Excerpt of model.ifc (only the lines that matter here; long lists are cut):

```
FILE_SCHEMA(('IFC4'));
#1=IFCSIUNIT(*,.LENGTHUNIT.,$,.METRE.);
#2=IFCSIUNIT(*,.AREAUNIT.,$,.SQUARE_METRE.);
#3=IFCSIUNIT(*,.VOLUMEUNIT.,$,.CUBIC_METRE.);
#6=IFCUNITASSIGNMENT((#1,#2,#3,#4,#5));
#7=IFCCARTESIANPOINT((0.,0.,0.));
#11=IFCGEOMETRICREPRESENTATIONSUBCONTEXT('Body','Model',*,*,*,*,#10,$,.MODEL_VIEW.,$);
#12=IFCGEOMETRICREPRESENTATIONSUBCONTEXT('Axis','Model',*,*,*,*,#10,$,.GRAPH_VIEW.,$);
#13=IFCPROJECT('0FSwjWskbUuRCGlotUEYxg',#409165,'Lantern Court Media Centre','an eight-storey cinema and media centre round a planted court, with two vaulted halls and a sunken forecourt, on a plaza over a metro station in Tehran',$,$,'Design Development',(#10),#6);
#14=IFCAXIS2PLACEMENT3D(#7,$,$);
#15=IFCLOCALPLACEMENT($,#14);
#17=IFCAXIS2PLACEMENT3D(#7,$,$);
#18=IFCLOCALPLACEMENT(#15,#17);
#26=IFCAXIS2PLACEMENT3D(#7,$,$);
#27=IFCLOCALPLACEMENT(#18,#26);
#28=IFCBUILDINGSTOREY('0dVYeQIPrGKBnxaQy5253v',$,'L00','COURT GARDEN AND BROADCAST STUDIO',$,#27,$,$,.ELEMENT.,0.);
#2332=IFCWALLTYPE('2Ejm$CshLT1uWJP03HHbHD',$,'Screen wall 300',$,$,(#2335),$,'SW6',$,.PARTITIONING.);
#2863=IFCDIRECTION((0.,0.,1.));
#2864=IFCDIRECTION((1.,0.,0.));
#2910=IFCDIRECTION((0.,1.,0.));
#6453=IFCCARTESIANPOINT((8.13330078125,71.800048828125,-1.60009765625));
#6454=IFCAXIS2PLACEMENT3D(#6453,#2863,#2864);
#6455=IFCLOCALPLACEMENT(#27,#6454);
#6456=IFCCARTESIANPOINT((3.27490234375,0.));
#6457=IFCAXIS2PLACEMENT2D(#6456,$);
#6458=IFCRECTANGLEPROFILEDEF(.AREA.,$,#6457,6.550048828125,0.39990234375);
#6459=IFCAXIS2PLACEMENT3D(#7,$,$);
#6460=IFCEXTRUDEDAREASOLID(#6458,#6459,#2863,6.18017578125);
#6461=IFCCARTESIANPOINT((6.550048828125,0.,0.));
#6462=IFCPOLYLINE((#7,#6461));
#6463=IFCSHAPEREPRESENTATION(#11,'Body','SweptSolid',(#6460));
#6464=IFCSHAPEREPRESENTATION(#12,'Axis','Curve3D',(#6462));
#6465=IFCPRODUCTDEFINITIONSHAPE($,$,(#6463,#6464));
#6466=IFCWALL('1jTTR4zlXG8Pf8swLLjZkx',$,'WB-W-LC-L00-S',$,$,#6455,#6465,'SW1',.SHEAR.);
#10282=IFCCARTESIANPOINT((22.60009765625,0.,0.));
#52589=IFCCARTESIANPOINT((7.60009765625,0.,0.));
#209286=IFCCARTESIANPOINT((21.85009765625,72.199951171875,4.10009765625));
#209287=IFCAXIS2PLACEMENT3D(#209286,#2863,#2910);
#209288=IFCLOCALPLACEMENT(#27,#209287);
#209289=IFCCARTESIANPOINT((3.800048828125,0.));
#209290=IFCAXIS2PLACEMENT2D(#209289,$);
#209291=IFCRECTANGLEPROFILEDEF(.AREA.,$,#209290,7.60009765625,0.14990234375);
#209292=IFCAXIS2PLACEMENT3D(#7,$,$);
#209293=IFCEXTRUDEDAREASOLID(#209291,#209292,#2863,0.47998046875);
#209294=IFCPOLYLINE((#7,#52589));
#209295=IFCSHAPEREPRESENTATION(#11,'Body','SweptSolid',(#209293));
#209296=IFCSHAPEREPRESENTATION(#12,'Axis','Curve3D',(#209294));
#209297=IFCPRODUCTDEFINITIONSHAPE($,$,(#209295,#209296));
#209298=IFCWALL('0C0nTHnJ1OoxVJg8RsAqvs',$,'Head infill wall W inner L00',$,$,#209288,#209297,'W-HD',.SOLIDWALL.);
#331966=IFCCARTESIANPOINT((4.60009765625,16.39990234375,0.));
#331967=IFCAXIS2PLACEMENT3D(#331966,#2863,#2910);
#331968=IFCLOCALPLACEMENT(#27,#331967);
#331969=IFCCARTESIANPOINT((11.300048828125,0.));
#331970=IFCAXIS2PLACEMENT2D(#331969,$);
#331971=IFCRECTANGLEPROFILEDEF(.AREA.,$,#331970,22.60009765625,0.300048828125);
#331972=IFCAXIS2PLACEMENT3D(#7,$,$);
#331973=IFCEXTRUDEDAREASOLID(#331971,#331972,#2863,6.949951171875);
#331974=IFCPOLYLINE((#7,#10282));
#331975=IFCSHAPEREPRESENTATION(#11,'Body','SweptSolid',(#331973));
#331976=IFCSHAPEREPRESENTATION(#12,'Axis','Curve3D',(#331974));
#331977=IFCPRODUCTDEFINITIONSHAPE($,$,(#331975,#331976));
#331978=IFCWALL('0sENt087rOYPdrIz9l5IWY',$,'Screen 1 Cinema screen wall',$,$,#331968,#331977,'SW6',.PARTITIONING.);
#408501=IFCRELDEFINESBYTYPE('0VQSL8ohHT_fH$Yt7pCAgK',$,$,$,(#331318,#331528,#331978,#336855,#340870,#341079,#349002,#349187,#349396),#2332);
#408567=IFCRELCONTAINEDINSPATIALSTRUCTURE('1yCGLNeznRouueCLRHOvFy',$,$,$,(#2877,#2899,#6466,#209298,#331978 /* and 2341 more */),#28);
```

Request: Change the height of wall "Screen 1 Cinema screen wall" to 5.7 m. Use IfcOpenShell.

```python
import ifcopenshell
import ifcopenshell.geom
import ifcopenshell.util.representation
import ifcopenshell.util.shape
import ifcopenshell.util.unit

model = ifcopenshell.open("model.ifc")
unit_scale = ifcopenshell.util.unit.calculate_unit_scale(model)
settings = ifcopenshell.geom.settings()


def volume(element):
    """Net volume in cubic metres, openings subtracted."""
    shape = ifcopenshell.geom.create_shape(settings, element)
    return ifcopenshell.util.shape.get_volume(shape.geometry)


wall = model.by_id(331978)
before = volume(wall)

body = ifcopenshell.util.representation.get_representation(wall, "Model", "Body")
solid = body.Items[0]
old_height = solid.Depth
solid.Depth = 5.7 / unit_scale
after = volume(wall)

print(f"height {old_height:g} -> {solid.Depth:g}, volume {before:.3f} -> {after:.3f} m3")

model.write("model_edited.ifc")
```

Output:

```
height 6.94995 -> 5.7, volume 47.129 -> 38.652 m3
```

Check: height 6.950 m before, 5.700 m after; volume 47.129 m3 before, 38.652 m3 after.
